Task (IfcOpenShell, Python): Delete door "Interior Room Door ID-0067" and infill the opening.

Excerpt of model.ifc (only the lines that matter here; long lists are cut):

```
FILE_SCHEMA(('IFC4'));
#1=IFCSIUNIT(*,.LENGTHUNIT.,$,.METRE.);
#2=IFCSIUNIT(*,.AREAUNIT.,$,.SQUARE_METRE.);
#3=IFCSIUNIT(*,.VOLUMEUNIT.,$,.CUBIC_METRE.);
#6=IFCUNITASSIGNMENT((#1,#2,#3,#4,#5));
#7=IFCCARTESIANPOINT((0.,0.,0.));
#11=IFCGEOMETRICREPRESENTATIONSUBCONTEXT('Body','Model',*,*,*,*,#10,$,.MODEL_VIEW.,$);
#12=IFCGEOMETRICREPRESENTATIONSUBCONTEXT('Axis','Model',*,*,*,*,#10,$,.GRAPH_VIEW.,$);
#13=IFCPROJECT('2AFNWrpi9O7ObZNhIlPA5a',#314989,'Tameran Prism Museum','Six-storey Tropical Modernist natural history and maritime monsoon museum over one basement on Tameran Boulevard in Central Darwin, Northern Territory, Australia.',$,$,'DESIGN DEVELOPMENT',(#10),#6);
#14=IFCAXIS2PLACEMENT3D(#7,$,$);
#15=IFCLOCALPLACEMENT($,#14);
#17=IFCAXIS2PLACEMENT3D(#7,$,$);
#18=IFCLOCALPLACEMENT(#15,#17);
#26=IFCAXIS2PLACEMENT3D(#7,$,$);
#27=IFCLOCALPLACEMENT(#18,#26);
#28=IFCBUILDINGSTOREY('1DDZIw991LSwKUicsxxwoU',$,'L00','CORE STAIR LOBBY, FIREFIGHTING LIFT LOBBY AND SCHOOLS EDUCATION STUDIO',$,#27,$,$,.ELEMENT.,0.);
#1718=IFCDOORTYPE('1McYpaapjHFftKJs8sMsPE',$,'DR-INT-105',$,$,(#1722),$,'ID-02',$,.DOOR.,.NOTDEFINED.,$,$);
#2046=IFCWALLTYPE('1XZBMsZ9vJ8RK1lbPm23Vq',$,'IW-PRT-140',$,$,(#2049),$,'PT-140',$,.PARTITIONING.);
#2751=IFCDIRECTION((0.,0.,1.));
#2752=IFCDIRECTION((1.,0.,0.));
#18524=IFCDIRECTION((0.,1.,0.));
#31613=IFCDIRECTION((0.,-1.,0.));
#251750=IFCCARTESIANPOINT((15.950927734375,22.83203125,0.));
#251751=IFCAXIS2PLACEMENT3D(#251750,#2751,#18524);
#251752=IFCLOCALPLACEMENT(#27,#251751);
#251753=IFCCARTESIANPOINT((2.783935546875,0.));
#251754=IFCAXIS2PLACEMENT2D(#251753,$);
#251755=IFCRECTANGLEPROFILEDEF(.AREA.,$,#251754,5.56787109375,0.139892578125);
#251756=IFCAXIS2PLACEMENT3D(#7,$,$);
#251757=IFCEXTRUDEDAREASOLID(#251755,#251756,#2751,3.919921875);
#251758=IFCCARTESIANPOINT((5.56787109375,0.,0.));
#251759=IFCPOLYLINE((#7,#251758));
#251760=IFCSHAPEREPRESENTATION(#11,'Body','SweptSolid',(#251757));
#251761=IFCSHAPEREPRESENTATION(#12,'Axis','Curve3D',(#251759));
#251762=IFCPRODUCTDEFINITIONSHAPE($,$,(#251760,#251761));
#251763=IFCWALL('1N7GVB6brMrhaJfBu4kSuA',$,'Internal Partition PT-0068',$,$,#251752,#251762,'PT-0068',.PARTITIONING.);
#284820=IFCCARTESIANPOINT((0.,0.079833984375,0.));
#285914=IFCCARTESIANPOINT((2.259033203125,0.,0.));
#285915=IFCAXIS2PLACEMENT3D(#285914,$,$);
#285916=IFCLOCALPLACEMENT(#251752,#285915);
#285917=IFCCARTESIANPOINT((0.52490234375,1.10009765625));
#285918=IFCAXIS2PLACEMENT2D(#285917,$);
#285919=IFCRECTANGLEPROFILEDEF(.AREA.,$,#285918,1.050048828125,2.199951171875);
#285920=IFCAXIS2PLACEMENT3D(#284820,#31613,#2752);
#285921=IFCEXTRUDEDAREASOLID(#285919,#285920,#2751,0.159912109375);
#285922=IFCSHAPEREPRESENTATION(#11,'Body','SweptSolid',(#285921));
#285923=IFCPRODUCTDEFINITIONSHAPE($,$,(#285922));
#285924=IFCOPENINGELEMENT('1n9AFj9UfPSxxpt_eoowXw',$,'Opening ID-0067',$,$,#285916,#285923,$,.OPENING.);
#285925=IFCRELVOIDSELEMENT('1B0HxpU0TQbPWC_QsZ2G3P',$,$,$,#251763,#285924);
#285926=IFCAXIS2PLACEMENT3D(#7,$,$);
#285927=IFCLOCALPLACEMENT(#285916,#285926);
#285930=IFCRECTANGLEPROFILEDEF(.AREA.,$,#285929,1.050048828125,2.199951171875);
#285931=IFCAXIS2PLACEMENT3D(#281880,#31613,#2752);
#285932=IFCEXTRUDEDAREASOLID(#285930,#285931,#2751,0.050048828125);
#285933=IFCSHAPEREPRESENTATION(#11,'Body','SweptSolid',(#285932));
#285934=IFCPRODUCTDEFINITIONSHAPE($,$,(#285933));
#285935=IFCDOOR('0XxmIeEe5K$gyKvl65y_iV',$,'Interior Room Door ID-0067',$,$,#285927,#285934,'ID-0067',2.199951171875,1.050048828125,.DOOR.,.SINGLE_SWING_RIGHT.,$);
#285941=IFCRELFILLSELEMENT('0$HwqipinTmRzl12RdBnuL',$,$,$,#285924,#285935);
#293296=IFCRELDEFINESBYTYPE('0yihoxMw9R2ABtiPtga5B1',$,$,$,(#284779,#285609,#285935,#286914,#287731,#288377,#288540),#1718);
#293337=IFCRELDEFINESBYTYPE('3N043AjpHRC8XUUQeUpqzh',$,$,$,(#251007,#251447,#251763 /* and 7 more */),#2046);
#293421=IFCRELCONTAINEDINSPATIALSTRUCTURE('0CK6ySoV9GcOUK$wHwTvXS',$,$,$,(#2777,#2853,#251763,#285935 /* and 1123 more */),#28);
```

```python
import ifcopenshell
import ifcopenshell.api.feature
import ifcopenshell.api.root
import ifcopenshell.geom
import ifcopenshell.util.shape

model = ifcopenshell.open("model.ifc")
settings = ifcopenshell.geom.settings()


def volume(element):
    """Net volume in cubic metres, openings subtracted."""
    shape = ifcopenshell.geom.create_shape(settings, element)
    return ifcopenshell.util.shape.get_volume(shape.geometry)


door = model.by_id(285935)
opening = door.FillsVoids[0].RelatingOpeningElement
wall = opening.VoidsElements[0].RelatingBuildingElement
before = volume(wall)

ifcopenshell.api.root.remove_product(model, product=door)
ifcopenshell.api.feature.remove_feature(model, feature=opening)

after = volume(wall)

print(f"wall volume {before:.3f} -> {after:.3f} m3")

model.write("model_v2.ifc")
```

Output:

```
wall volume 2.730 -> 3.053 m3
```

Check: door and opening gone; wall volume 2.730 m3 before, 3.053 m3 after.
